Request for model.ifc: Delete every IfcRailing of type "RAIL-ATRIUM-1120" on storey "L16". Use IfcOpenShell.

First a look at what the model holds.

```python
import ifcopenshell
import ifcopenshell.util.element

model = ifcopenshell.open("model.ifc")
print(model.schema)
storey = next(s for s in model.by_type("IfcBuildingStorey") if s.Name == "L16")
railings = [e for e in ifcopenshell.util.element.get_decomposition(storey) if e.is_a("IfcRailing")]
seen = {}
for e in railings:
    element_type = ifcopenshell.util.element.get_type(e)
    name = element_type.Name if element_type not in (None, e) else None
    seen[name] = seen.get(name, 0) + 1
for name, count in sorted(seen.items(), key=str):
    print(count, "x", name)
```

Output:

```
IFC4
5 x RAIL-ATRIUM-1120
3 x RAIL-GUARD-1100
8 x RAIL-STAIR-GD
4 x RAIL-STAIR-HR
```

```python
import ifcopenshell
import ifcopenshell.api.root
import ifcopenshell.util.element

model = ifcopenshell.open("model.ifc")

storey = next(s for s in model.by_type("IfcBuildingStorey") if s.Name == "L16")
railings = [e for e in ifcopenshell.util.element.get_decomposition(storey) if e.is_a("IfcRailing")]
targets = [e for e in railings if (t := ifcopenshell.util.element.get_type(e)) not in (None, e) and t.Name == "RAIL-ATRIUM-1120"]

for e in targets:
    ifcopenshell.api.root.remove_product(model, product=e)
print(len(targets), "removed")

model.write("model-out.ifc")
```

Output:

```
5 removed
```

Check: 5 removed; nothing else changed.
